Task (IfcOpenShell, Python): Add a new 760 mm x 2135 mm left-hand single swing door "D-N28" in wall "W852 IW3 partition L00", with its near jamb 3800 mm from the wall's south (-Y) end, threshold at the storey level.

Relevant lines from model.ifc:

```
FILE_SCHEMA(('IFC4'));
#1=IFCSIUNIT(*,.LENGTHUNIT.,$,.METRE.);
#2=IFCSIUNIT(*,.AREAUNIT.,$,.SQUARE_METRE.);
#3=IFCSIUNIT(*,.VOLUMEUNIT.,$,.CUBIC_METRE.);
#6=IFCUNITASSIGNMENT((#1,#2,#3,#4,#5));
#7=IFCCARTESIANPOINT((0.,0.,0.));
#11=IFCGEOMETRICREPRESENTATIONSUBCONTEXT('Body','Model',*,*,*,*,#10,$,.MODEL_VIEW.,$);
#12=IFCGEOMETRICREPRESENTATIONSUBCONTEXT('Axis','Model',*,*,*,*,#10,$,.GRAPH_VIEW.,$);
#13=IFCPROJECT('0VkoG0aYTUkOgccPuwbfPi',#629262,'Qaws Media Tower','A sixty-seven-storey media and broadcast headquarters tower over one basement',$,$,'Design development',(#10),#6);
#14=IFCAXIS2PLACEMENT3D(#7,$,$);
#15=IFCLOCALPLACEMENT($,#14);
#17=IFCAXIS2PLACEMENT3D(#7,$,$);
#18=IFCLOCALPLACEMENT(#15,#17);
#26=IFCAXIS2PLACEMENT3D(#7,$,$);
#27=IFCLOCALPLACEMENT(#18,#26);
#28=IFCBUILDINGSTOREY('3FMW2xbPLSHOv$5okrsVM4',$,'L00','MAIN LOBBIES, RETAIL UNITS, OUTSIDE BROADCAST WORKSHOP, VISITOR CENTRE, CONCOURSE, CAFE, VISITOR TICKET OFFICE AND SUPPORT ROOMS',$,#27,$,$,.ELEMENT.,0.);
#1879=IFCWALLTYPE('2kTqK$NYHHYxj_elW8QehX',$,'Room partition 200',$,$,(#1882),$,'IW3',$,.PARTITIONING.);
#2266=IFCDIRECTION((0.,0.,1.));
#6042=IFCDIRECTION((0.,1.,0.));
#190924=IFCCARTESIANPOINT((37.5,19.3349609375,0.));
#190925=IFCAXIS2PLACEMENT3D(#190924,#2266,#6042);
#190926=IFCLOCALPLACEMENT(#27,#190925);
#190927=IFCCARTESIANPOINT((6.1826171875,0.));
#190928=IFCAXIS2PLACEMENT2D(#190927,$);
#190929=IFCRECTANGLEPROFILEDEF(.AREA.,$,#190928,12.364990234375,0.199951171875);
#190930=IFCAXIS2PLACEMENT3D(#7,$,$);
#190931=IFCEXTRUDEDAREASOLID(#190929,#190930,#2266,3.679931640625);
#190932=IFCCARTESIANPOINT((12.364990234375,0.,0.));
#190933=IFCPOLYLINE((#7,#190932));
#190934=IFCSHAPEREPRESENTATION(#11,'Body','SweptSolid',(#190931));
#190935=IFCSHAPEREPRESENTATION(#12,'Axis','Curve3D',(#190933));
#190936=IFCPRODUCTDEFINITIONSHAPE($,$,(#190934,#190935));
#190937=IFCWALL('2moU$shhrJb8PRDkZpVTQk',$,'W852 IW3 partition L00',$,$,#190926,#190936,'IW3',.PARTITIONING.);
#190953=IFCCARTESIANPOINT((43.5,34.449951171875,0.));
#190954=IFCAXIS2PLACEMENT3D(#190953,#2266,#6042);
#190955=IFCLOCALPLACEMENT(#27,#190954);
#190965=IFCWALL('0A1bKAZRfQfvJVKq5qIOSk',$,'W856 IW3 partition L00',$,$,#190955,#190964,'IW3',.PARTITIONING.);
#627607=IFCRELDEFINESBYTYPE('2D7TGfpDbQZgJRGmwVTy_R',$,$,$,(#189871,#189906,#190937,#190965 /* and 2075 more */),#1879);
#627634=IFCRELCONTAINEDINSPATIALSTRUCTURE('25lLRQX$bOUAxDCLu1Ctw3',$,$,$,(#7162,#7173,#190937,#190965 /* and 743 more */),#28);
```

```python
import numpy as np
import ifcopenshell
import ifcopenshell.api.feature
import ifcopenshell.api.geometry
import ifcopenshell.api.root
import ifcopenshell.api.spatial
import ifcopenshell.geom
import ifcopenshell.util.element
import ifcopenshell.util.placement
import ifcopenshell.util.representation
import ifcopenshell.util.shape
import ifcopenshell.util.unit

model = ifcopenshell.open("model.ifc")
unit_scale = ifcopenshell.util.unit.calculate_unit_scale(model)
settings = ifcopenshell.geom.settings()


def volume(element):
    """Net volume in cubic metres, openings subtracted."""
    shape = ifcopenshell.geom.create_shape(settings, element)
    return ifcopenshell.util.shape.get_volume(shape.geometry)


wall = model.by_guid("2moU$shhrJb8PRDkZpVTQk")
storey = ifcopenshell.util.element.get_container(wall, ifc_class="IfcBuildingStorey")
context = ifcopenshell.util.representation.get_context(model, "Model", "Body", "MODEL_VIEW")
before = volume(wall)

width, height, from_end, sill = 0.76, 2.135, 3.8, 0.0  # metres

# The wall runs along its own X axis, and the end named is its -X end.
wall_shape = ifcopenshell.geom.create_shape(settings, wall)
x, y, z = ifcopenshell.util.shape.get_vertices(wall_shape.geometry).T
start = x.min() + from_end
face, thickness = float(y.min()), float(y.max() - y.min())
wall_matrix = ifcopenshell.util.placement.get_local_placement(wall.ObjectPlacement)
level = ifcopenshell.util.placement.get_local_placement(storey.ObjectPlacement)[2, 3]


def in_wall(x, y):
    """Placement at x, y metres in the wall's axes, at sill height."""
    matrix = wall_matrix.copy()
    matrix[:, 3] = wall_matrix @ np.array([x / unit_scale, y / unit_scale, 0.0, 1.0])
    matrix[2, 3] = level + sill / unit_scale
    return matrix


# Opening: a box that overshoots both wall faces by 50 mm.
opening = ifcopenshell.api.root.create_entity(model, ifc_class="IfcOpeningElement", predefined_type="OPENING")
box = ifcopenshell.api.geometry.add_wall_representation(
    model, context=context, length=width, height=height, thickness=thickness + 0.1
)
ifcopenshell.api.geometry.assign_representation(model, product=opening, representation=box)
ifcopenshell.api.geometry.edit_object_placement(model, product=opening, matrix=in_wall(start, face - 0.05), is_si=False)
ifcopenshell.api.feature.add_feature(model, feature=opening, element=wall)

door = ifcopenshell.api.root.create_entity(model, ifc_class="IfcDoor", name="D-N28", predefined_type="DOOR")
door.OverallWidth, door.OverallHeight = width / unit_scale, height / unit_scale
door.OperationType = "SINGLE_SWING_LEFT"
body = ifcopenshell.api.geometry.add_door_representation(
    model,
    context=context,
    overall_width=door.OverallWidth,
    overall_height=door.OverallHeight,
    operation_type="SINGLE_SWING_LEFT",
    lining_properties={"LiningDepth": thickness / unit_scale, "ThresholdDepth": thickness / unit_scale},
)
ifcopenshell.api.geometry.assign_representation(model, product=door, representation=body)
ifcopenshell.api.spatial.assign_container(model, products=[door], relating_structure=storey)
ifcopenshell.api.feature.add_filling(model, opening=opening, element=door)

# The lining spans the wall, so the door starts at the wall face.
ifcopenshell.api.geometry.edit_object_placement(model, product=door, matrix=in_wall(start, face), is_si=False)

after = volume(wall)

print(f"wall volume {before:.3f} -> {after:.3f} m3")

model.write("model_rev.ifc")
```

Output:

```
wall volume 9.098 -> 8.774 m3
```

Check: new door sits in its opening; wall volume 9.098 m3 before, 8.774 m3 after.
